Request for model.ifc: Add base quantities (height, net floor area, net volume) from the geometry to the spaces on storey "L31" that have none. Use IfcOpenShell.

First a look at what the model holds.

```python
import ifcopenshell
import ifcopenshell.util.element
import ifcopenshell.util.unit

model = ifcopenshell.open("model.ifc")
print(model.schema)
for unit_type in ("LENGTHUNIT", "AREAUNIT", "VOLUMEUNIT"):
    print(unit_type, ifcopenshell.util.unit.calculate_unit_scale(model, unit_type))
storey = next(s for s in model.by_type("IfcBuildingStorey") if s.Name == "L31")
spaces = [e for e in ifcopenshell.util.element.get_decomposition(storey) if e.is_a("IfcSpace")]
for e in sorted(spaces, key=lambda e: e.id()):
    print(e.id(), e.is_a(), e.Name, list(ifcopenshell.util.element.get_psets(e, qtos_only=True)), sep=" | ")
```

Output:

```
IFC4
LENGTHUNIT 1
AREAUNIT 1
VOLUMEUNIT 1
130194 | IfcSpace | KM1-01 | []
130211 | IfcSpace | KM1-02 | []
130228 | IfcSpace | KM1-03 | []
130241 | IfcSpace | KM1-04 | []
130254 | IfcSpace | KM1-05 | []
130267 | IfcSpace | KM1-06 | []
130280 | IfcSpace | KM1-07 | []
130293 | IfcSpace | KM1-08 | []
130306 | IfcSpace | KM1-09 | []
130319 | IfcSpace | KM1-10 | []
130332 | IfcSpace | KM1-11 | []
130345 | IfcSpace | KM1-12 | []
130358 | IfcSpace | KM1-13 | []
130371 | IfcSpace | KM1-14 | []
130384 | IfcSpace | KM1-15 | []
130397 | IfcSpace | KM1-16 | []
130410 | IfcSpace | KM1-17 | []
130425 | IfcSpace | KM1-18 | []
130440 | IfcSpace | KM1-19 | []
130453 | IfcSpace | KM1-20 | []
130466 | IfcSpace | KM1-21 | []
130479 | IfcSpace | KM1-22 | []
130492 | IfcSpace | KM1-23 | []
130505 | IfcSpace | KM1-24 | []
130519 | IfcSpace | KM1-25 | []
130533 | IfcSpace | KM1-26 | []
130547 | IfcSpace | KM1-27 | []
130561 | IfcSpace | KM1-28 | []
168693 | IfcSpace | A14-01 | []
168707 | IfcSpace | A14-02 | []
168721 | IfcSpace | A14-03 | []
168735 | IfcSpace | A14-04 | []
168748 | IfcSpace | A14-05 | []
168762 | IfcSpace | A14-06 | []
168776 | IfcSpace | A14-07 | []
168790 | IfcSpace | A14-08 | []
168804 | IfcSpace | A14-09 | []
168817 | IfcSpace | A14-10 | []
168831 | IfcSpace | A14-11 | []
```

```python
import ifcopenshell
import ifcopenshell.api.pset
import ifcopenshell.geom
import ifcopenshell.util.element
import ifcopenshell.util.shape
import ifcopenshell.util.unit

model = ifcopenshell.open("model.ifc")
unit_scale = ifcopenshell.util.unit.calculate_unit_scale(model)
area_scale = ifcopenshell.util.unit.calculate_unit_scale(model, "AREAUNIT")
volume_scale = ifcopenshell.util.unit.calculate_unit_scale(model, "VOLUMEUNIT")
settings = ifcopenshell.geom.settings()

storey = next(s for s in model.by_type("IfcBuildingStorey") if s.Name == "L31")
spaces = [e for e in ifcopenshell.util.element.get_decomposition(storey) if e.is_a("IfcSpace")]

for e in sorted(spaces, key=lambda e: e.id()):
    if ifcopenshell.util.element.get_psets(e, qtos_only=True, should_inherit=False):
        continue
    # Geometry comes back in metres, in the element's own axes.
    shape = ifcopenshell.geom.create_shape(settings, e)
    values = {
        "Height": ifcopenshell.util.shape.get_z(shape.geometry) / unit_scale,
        "NetFloorArea": ifcopenshell.util.shape.get_footprint_area(shape.geometry) / area_scale,
        "NetVolume": ifcopenshell.util.shape.get_volume(shape.geometry) / volume_scale,
    }
    qto = ifcopenshell.api.pset.add_qto(model, product=e, name="Qto_SpaceBaseQuantities")
    ifcopenshell.api.pset.edit_qto(model, qto=qto, properties=values)
    print(e.id(), {k: round(v, 3) for k, v in values.items()})

model.write("model_updated.ifc")
```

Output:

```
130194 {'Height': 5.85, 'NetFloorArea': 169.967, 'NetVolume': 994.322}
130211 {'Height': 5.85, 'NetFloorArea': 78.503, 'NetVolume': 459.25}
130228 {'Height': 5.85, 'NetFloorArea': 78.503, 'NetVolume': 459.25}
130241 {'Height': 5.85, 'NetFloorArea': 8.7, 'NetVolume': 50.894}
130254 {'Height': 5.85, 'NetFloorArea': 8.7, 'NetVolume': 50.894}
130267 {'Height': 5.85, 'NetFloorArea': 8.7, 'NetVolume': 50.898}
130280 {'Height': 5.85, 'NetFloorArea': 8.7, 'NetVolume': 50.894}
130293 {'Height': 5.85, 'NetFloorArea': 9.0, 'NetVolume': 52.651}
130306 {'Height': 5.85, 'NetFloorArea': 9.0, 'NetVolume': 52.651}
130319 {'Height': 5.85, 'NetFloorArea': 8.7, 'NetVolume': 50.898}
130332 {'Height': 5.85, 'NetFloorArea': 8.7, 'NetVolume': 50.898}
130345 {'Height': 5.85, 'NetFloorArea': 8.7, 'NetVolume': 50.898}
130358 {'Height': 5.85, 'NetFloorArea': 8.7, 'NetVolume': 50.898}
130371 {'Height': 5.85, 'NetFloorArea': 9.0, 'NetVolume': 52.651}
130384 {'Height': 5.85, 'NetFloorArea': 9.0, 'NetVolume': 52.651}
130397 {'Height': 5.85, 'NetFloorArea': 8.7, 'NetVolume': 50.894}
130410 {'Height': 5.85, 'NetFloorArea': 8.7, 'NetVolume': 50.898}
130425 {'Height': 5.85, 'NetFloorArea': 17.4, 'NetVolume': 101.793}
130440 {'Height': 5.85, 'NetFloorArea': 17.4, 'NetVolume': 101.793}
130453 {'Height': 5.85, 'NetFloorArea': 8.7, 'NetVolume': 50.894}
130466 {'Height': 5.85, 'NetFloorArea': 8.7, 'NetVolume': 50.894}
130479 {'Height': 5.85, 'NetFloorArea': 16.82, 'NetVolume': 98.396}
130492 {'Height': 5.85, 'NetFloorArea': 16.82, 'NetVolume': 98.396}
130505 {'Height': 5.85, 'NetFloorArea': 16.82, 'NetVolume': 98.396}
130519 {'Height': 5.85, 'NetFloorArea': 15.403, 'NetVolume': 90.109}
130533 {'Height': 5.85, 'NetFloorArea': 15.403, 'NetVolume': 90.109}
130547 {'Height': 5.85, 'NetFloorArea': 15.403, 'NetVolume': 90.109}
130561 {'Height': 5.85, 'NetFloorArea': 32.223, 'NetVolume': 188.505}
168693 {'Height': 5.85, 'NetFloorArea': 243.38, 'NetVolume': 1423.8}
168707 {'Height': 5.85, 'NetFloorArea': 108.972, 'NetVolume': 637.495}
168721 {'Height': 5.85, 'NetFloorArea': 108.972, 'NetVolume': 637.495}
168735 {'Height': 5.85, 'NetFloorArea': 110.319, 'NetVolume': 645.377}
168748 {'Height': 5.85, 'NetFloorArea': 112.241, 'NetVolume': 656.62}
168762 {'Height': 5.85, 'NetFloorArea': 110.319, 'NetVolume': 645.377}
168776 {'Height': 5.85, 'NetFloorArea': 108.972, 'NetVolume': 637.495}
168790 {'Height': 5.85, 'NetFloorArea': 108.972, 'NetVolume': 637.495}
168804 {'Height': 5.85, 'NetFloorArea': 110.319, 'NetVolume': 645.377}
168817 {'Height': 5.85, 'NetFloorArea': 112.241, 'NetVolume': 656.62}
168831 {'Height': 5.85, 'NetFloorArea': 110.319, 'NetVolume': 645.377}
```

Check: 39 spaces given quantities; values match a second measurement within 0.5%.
